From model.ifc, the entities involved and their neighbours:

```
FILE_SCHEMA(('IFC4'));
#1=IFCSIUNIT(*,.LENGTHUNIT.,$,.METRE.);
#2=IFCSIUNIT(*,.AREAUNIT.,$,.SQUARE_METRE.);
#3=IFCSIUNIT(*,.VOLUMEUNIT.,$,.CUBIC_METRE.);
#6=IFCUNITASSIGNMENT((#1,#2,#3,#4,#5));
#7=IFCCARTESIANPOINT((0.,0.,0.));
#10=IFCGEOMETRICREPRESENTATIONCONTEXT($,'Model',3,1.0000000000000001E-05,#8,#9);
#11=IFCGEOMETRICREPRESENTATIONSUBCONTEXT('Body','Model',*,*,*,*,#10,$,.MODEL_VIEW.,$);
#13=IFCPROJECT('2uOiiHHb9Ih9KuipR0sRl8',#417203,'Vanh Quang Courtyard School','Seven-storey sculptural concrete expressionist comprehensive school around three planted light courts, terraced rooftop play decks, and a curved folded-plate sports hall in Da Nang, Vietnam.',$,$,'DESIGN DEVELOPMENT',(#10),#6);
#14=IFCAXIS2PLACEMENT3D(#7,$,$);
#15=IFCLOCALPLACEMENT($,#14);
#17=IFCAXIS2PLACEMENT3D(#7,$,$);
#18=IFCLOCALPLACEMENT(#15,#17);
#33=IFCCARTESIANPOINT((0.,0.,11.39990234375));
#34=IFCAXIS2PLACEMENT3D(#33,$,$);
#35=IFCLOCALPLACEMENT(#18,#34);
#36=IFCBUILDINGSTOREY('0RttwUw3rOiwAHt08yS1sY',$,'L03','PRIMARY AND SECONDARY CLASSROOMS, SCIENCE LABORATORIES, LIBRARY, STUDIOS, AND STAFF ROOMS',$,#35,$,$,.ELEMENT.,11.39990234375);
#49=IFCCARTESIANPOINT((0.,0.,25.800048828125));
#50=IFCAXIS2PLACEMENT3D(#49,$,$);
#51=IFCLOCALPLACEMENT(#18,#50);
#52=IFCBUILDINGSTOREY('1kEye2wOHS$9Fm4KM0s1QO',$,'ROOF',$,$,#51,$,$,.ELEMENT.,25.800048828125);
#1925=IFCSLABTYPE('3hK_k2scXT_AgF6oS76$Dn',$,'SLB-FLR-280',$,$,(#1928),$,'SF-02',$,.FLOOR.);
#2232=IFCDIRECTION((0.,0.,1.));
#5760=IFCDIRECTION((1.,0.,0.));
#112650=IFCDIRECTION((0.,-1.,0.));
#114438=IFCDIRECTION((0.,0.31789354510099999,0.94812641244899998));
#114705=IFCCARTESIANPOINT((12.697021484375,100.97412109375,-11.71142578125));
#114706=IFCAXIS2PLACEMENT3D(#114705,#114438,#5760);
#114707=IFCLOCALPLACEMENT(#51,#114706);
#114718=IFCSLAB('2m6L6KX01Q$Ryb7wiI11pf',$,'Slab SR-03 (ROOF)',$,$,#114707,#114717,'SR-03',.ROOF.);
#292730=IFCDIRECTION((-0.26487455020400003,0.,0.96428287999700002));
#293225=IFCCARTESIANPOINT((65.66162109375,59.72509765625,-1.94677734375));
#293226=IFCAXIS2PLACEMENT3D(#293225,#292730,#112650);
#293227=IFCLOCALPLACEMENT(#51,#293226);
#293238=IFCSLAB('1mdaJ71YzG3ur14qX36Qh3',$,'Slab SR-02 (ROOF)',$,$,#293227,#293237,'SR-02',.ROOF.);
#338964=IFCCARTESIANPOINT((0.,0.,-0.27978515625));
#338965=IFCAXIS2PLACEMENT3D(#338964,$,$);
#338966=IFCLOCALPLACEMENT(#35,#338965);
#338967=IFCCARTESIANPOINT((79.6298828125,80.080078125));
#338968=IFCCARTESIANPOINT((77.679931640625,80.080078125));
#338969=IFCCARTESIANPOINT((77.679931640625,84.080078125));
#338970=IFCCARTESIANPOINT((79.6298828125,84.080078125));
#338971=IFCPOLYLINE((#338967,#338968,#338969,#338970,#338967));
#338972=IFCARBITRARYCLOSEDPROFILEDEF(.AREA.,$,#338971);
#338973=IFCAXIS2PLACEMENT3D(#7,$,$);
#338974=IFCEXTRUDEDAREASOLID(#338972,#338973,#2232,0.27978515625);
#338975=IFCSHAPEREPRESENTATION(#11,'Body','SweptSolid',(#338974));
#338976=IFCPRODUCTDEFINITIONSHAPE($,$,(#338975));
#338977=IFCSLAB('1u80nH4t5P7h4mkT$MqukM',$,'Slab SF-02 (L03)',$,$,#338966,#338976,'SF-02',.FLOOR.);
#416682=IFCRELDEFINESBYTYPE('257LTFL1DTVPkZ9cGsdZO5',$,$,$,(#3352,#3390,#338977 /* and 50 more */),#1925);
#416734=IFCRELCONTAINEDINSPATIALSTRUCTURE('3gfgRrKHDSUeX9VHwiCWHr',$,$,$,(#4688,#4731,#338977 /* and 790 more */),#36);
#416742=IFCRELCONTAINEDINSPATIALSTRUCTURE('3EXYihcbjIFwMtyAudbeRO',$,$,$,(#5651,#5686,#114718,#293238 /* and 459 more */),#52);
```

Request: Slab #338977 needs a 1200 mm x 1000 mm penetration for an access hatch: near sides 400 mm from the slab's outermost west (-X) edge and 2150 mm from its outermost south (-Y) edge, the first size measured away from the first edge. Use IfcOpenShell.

```python
import numpy as np
import ifcopenshell
import ifcopenshell.api.feature
import ifcopenshell.api.geometry
import ifcopenshell.api.root
import ifcopenshell.geom
import ifcopenshell.util.placement
import ifcopenshell.util.representation
import ifcopenshell.util.shape
import ifcopenshell.util.unit

model = ifcopenshell.open("model.ifc")
unit_scale = ifcopenshell.util.unit.calculate_unit_scale(model)
settings = ifcopenshell.geom.settings()


def volume(element):
    """Net volume in cubic metres, openings subtracted."""
    shape = ifcopenshell.geom.create_shape(settings, element)
    return ifcopenshell.util.shape.get_volume(shape.geometry)


slab = model.by_guid("1u80nH4t5P7h4mkT$MqukM")
before = volume(slab)

# Extent in the slab's own axes, in metres. The edges named are its -X and -Y sides.
slab_shape = ifcopenshell.geom.create_shape(settings, slab)
vertices = ifcopenshell.util.shape.get_vertices(slab_shape.geometry)
x_min, y_min, bottom = vertices.min(axis=0)
top = vertices[:, 2].max()

opening = ifcopenshell.api.root.create_entity(model, ifc_class="IfcOpeningElement", name="Access hatch opening", predefined_type="OPENING")
context = ifcopenshell.util.representation.get_context(model, "Model", "Body", "MODEL_VIEW")
width, depth = 1.2, 1
outline = [(0.0, 0.0), (width, 0.0), (width, depth), (0.0, depth), (0.0, 0.0)]
# Overshoot both faces by 50 mm so the cut is clean.
shape = ifcopenshell.api.geometry.add_slab_representation(
    model, context=context, depth=top - bottom + 0.1, polyline=outline
)
ifcopenshell.api.geometry.assign_representation(model, product=opening, representation=shape)

matrix = ifcopenshell.util.placement.get_local_placement(slab.ObjectPlacement)
matrix[:, 3] = matrix @ np.append(np.array([x_min + 0.4, y_min + 2.15, bottom - 0.05]) / unit_scale, 1.0)
ifcopenshell.api.geometry.edit_object_placement(model, product=opening, matrix=matrix, is_si=False)
ifcopenshell.api.feature.add_feature(model, feature=opening, element=slab)

after = volume(slab)

print(f"slab volume {before:.3f} -> {after:.3f} m3")

model.write("model_edited.ifc")
```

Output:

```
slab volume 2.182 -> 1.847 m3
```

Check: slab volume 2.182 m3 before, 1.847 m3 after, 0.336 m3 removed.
